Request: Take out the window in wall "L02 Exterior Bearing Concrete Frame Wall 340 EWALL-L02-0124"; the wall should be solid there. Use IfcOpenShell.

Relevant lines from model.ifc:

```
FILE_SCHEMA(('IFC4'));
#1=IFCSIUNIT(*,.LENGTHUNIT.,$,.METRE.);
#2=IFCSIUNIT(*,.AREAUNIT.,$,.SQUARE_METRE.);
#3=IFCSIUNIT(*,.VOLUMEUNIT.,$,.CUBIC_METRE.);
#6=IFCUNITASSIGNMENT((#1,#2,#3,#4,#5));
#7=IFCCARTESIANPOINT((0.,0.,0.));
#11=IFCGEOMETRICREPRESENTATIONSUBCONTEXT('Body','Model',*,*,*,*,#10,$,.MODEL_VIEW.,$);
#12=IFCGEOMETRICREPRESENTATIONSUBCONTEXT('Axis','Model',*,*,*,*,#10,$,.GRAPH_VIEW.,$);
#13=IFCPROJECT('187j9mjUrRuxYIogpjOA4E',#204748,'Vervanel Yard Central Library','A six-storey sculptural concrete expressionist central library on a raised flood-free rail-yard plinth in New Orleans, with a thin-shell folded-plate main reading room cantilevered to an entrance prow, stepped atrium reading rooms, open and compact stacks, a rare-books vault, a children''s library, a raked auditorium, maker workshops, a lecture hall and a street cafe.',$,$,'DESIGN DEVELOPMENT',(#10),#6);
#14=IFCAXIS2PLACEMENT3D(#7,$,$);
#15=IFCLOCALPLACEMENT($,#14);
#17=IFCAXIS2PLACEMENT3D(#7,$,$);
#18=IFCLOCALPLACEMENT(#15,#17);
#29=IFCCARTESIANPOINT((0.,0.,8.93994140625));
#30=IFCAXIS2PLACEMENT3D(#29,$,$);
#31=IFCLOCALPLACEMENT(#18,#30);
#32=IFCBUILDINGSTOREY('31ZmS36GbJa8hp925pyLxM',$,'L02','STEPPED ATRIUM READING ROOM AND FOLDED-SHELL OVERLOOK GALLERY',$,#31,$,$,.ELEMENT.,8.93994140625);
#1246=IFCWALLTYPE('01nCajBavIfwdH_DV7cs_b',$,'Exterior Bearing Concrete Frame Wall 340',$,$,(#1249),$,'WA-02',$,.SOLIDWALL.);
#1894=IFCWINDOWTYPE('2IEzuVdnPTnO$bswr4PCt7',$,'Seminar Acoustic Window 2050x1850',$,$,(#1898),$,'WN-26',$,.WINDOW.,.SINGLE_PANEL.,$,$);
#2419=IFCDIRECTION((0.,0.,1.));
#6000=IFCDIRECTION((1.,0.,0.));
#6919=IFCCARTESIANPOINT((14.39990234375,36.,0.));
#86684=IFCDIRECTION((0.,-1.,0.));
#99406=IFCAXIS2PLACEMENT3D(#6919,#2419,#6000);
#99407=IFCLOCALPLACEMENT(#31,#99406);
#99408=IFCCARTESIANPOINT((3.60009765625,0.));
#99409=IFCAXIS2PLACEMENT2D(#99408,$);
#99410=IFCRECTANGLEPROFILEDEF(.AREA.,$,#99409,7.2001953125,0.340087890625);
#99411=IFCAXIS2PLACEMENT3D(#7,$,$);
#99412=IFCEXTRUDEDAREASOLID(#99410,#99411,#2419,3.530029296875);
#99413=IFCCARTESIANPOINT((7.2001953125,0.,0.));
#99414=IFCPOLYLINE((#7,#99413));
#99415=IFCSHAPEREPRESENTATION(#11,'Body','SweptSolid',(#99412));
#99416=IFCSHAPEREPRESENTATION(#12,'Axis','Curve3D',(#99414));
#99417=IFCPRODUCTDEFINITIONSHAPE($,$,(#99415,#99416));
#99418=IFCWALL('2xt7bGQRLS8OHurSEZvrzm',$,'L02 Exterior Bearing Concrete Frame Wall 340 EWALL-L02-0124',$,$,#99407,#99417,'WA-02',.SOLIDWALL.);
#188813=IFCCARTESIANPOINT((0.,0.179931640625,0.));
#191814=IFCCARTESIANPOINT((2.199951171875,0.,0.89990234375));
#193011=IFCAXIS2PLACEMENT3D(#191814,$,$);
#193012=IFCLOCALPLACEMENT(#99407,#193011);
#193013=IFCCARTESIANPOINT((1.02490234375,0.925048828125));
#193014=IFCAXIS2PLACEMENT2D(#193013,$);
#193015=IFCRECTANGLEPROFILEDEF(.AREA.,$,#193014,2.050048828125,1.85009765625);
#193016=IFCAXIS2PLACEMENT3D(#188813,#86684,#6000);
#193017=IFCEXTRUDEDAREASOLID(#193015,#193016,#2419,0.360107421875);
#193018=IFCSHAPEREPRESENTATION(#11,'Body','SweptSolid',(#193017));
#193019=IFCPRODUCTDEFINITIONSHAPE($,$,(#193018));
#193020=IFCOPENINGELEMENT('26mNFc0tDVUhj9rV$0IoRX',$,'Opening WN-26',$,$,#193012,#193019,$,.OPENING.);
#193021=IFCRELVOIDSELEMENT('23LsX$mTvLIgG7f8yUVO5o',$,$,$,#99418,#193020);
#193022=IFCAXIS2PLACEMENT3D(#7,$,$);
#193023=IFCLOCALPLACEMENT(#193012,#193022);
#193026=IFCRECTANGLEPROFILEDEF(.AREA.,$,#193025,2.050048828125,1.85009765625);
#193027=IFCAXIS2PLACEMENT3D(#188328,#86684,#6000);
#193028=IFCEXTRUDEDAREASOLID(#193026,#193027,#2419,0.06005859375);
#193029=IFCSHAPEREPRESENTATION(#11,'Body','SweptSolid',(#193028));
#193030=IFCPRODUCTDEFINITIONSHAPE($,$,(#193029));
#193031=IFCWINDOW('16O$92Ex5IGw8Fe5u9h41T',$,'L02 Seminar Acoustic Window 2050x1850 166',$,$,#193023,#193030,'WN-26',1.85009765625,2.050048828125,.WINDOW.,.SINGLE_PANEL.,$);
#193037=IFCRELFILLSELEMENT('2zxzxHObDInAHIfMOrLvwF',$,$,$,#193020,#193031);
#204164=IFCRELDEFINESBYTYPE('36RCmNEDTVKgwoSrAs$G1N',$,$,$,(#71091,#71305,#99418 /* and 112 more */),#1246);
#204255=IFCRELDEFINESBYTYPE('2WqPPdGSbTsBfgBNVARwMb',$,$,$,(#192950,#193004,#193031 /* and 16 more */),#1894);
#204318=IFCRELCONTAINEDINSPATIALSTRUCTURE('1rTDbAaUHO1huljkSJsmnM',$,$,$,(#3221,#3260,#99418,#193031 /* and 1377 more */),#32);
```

```python
import ifcopenshell
import ifcopenshell.api.feature
import ifcopenshell.api.root
import ifcopenshell.geom
import ifcopenshell.util.shape

model = ifcopenshell.open("model.ifc")
settings = ifcopenshell.geom.settings()


def volume(element):
    """Net volume in cubic metres, openings subtracted."""
    shape = ifcopenshell.geom.create_shape(settings, element)
    return ifcopenshell.util.shape.get_volume(shape.geometry)


window = model.by_id(193031)
opening = window.FillsVoids[0].RelatingOpeningElement
wall = opening.VoidsElements[0].RelatingBuildingElement
before = volume(wall)

ifcopenshell.api.root.remove_product(model, product=window)
ifcopenshell.api.feature.remove_feature(model, feature=opening)

after = volume(wall)

print(f"wall volume {before:.3f} -> {after:.3f} m3")

model.write("model_edited.ifc")
```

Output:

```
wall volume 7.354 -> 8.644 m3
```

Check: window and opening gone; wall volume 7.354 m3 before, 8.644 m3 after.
